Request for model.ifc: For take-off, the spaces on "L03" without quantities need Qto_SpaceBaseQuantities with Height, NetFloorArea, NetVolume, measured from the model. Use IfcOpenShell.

First a look at what the model holds.

```python
import ifcopenshell
import ifcopenshell.util.element
import ifcopenshell.util.unit

model = ifcopenshell.open("model.ifc")
print(model.schema)
for unit_type in ("LENGTHUNIT", "AREAUNIT", "VOLUMEUNIT"):
    print(unit_type, ifcopenshell.util.unit.calculate_unit_scale(model, unit_type))
storey = next(s for s in model.by_type("IfcBuildingStorey") if s.Name == "L03")
spaces = [e for e in ifcopenshell.util.element.get_decomposition(storey) if e.is_a("IfcSpace")]
for e in sorted(spaces, key=lambda e: e.id()):
    print(e.id(), e.is_a(), e.Name, list(ifcopenshell.util.element.get_psets(e, qtos_only=True)), sep=" | ")
```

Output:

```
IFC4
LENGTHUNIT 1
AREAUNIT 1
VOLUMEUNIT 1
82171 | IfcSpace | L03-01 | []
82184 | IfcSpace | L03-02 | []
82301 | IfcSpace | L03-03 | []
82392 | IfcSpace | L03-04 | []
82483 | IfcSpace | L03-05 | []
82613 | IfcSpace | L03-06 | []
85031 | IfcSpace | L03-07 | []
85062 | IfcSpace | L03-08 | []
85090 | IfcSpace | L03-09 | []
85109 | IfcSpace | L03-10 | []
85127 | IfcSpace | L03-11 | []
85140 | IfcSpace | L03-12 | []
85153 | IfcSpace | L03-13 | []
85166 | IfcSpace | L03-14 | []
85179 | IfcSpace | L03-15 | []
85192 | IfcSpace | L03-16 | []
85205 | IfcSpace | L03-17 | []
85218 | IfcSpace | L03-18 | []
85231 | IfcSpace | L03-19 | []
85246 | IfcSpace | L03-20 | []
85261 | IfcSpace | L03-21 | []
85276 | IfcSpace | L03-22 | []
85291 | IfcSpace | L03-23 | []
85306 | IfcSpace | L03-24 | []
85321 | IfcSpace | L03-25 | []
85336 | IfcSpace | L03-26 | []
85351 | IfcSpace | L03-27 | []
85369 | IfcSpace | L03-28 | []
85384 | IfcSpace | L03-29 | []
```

```python
import ifcopenshell
import ifcopenshell.api.pset
import ifcopenshell.geom
import ifcopenshell.util.element
import ifcopenshell.util.shape
import ifcopenshell.util.unit

model = ifcopenshell.open("model.ifc")
unit_scale = ifcopenshell.util.unit.calculate_unit_scale(model)
area_scale = ifcopenshell.util.unit.calculate_unit_scale(model, "AREAUNIT")
volume_scale = ifcopenshell.util.unit.calculate_unit_scale(model, "VOLUMEUNIT")
settings = ifcopenshell.geom.settings()

storey = next(s for s in model.by_type("IfcBuildingStorey") if s.Name == "L03")
spaces = [e for e in ifcopenshell.util.element.get_decomposition(storey) if e.is_a("IfcSpace")]

for e in sorted(spaces, key=lambda e: e.id()):
    if ifcopenshell.util.element.get_psets(e, qtos_only=True, should_inherit=False):
        continue
    # Geometry comes back in metres, in the element's own axes.
    shape = ifcopenshell.geom.create_shape(settings, e)
    values = {
        "Height": ifcopenshell.util.shape.get_z(shape.geometry) / unit_scale,
        "NetFloorArea": ifcopenshell.util.shape.get_footprint_area(shape.geometry) / area_scale,
        "NetVolume": ifcopenshell.util.shape.get_volume(shape.geometry) / volume_scale,
    }
    qto = ifcopenshell.api.pset.add_qto(model, product=e, name="Qto_SpaceBaseQuantities")
    ifcopenshell.api.pset.edit_qto(model, qto=qto, properties=values)
    print(e.id(), {k: round(v, 3) for k, v in values.items()})

model.write("model_rev.ifc")
```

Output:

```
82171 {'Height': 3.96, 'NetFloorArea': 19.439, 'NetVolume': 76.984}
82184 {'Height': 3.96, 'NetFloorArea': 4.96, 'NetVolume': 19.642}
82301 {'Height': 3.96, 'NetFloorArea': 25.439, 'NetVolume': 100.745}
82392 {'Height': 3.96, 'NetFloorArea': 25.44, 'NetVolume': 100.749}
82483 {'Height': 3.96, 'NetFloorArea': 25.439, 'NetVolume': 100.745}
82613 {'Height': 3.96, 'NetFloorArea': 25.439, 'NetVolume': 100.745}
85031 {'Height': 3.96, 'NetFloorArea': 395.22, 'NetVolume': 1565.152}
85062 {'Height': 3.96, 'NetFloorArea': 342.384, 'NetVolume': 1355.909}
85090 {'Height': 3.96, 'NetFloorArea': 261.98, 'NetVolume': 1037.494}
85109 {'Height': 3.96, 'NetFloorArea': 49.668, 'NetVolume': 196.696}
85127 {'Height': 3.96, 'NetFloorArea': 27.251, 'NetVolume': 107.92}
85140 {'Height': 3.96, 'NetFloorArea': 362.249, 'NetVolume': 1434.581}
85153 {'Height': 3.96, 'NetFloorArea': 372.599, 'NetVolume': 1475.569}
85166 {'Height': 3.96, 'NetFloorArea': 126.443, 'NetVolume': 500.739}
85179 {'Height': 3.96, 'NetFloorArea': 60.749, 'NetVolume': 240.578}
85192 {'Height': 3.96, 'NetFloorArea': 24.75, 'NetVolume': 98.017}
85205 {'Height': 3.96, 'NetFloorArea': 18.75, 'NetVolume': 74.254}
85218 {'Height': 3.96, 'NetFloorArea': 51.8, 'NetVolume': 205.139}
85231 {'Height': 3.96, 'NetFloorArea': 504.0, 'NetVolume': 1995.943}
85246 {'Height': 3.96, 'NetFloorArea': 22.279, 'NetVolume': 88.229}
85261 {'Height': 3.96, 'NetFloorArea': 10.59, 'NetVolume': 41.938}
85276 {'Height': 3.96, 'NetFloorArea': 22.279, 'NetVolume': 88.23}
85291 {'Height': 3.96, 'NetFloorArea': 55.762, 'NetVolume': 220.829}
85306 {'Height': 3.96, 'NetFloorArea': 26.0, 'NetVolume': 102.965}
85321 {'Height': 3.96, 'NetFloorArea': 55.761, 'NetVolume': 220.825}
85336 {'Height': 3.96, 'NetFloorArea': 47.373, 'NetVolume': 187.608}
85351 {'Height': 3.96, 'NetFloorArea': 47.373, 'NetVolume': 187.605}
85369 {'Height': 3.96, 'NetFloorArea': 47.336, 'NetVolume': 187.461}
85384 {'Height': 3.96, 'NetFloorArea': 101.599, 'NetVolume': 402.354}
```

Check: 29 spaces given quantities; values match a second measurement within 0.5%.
